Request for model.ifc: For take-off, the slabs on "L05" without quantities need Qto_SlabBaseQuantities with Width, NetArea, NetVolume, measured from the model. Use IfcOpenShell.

First a look at what the model holds.

```python
import ifcopenshell
import ifcopenshell.util.element
import ifcopenshell.util.unit

model = ifcopenshell.open("model.ifc")
print(model.schema)
for unit_type in ("LENGTHUNIT", "AREAUNIT", "VOLUMEUNIT"):
    print(unit_type, ifcopenshell.util.unit.calculate_unit_scale(model, unit_type))
storey = next(s for s in model.by_type("IfcBuildingStorey") if s.Name == "L05")
slabs = [e for e in ifcopenshell.util.element.get_decomposition(storey) if e.is_a("IfcSlab")]
for e in sorted(slabs, key=lambda e: e.id()):
    print(e.id(), e.is_a(), e.Name, list(ifcopenshell.util.element.get_psets(e, qtos_only=True)), sep=" | ")
```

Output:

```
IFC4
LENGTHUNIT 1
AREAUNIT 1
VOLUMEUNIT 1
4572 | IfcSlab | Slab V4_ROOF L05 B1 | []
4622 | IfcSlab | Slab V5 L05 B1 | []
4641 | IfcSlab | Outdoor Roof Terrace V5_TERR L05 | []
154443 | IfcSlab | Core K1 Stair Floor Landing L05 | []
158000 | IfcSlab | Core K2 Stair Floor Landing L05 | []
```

```python
import ifcopenshell
import ifcopenshell.api.pset
import ifcopenshell.geom
import ifcopenshell.util.element
import ifcopenshell.util.shape
import ifcopenshell.util.unit

model = ifcopenshell.open("model.ifc")
unit_scale = ifcopenshell.util.unit.calculate_unit_scale(model)
area_scale = ifcopenshell.util.unit.calculate_unit_scale(model, "AREAUNIT")
volume_scale = ifcopenshell.util.unit.calculate_unit_scale(model, "VOLUMEUNIT")
settings = ifcopenshell.geom.settings()

storey = next(s for s in model.by_type("IfcBuildingStorey") if s.Name == "L05")
slabs = [e for e in ifcopenshell.util.element.get_decomposition(storey) if e.is_a("IfcSlab")]

for e in sorted(slabs, key=lambda e: e.id()):
    if ifcopenshell.util.element.get_psets(e, qtos_only=True, should_inherit=False):
        continue
    # Geometry comes back in metres, in the element's own axes.
    shape = ifcopenshell.geom.create_shape(settings, e)
    values = {
        "Width": ifcopenshell.util.shape.get_z(shape.geometry) / unit_scale,
        "NetArea": ifcopenshell.util.shape.get_footprint_area(shape.geometry) / area_scale,
        "NetVolume": ifcopenshell.util.shape.get_volume(shape.geometry) / volume_scale,
    }
    qto = ifcopenshell.api.pset.add_qto(model, product=e, name="Qto_SlabBaseQuantities")
    ifcopenshell.api.pset.edit_qto(model, qto=qto, properties=values)
    print(e.id(), {k: round(v, 3) for k, v in values.items()})

model.write("model_updated.ifc")
```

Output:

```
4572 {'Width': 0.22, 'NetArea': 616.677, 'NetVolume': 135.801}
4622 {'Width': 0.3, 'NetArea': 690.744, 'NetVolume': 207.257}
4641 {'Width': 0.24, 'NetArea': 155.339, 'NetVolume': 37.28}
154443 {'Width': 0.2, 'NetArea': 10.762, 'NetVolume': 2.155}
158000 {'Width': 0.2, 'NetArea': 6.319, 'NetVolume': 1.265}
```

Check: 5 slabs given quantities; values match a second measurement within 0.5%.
